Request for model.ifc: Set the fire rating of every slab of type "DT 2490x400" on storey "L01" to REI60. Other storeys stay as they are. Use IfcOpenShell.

First a look at what the model holds.

```python
import ifcopenshell
import ifcopenshell.util.element

model = ifcopenshell.open("model.ifc")
print(model.schema)
storey = next(s for s in model.by_type("IfcBuildingStorey") if s.Name == "L01")
slabs = [e for e in ifcopenshell.util.element.get_decomposition(storey) if e.is_a("IfcSlab")]
seen = {}
for e in slabs:
    element_type = ifcopenshell.util.element.get_type(e)
    key = (element_type.Name if element_type != e and element_type else None, ifcopenshell.util.element.get_pset(e, "Pset_SlabCommon", "FireRating"))
    seen[key] = seen.get(key, 0) + 1
for (name, value), count in sorted(seen.items(), key=str):
    print(count, "x", name, "|", value)
```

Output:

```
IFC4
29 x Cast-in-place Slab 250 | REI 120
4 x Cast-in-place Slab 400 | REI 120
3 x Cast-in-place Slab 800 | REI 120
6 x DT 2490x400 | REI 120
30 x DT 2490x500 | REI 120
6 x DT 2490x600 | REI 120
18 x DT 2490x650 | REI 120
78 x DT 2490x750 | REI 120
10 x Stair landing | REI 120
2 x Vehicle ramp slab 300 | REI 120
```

```python
import ifcopenshell
import ifcopenshell.api.pset
import ifcopenshell.util.element

model = ifcopenshell.open("model.ifc")

storey = next(s for s in model.by_type("IfcBuildingStorey") if s.Name == "L01")
slabs = [e for e in ifcopenshell.util.element.get_decomposition(storey) if e.is_a("IfcSlab")]

count = 0
for e in slabs:
    element_type = ifcopenshell.util.element.get_type(e)
    if element_type in (None, e) or element_type.Name != "DT 2490x400":
        continue
    # add_pset returns the element's existing set when there is one.
    pset = ifcopenshell.api.pset.add_pset(model, product=e, name="Pset_SlabCommon")
    ifcopenshell.api.pset.edit_pset(model, pset=pset, properties={"FireRating": "REI60"})
    count += 1

print(count, "slabs updated")

model.write("model_edited.ifc")
```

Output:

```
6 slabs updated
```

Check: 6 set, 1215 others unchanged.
